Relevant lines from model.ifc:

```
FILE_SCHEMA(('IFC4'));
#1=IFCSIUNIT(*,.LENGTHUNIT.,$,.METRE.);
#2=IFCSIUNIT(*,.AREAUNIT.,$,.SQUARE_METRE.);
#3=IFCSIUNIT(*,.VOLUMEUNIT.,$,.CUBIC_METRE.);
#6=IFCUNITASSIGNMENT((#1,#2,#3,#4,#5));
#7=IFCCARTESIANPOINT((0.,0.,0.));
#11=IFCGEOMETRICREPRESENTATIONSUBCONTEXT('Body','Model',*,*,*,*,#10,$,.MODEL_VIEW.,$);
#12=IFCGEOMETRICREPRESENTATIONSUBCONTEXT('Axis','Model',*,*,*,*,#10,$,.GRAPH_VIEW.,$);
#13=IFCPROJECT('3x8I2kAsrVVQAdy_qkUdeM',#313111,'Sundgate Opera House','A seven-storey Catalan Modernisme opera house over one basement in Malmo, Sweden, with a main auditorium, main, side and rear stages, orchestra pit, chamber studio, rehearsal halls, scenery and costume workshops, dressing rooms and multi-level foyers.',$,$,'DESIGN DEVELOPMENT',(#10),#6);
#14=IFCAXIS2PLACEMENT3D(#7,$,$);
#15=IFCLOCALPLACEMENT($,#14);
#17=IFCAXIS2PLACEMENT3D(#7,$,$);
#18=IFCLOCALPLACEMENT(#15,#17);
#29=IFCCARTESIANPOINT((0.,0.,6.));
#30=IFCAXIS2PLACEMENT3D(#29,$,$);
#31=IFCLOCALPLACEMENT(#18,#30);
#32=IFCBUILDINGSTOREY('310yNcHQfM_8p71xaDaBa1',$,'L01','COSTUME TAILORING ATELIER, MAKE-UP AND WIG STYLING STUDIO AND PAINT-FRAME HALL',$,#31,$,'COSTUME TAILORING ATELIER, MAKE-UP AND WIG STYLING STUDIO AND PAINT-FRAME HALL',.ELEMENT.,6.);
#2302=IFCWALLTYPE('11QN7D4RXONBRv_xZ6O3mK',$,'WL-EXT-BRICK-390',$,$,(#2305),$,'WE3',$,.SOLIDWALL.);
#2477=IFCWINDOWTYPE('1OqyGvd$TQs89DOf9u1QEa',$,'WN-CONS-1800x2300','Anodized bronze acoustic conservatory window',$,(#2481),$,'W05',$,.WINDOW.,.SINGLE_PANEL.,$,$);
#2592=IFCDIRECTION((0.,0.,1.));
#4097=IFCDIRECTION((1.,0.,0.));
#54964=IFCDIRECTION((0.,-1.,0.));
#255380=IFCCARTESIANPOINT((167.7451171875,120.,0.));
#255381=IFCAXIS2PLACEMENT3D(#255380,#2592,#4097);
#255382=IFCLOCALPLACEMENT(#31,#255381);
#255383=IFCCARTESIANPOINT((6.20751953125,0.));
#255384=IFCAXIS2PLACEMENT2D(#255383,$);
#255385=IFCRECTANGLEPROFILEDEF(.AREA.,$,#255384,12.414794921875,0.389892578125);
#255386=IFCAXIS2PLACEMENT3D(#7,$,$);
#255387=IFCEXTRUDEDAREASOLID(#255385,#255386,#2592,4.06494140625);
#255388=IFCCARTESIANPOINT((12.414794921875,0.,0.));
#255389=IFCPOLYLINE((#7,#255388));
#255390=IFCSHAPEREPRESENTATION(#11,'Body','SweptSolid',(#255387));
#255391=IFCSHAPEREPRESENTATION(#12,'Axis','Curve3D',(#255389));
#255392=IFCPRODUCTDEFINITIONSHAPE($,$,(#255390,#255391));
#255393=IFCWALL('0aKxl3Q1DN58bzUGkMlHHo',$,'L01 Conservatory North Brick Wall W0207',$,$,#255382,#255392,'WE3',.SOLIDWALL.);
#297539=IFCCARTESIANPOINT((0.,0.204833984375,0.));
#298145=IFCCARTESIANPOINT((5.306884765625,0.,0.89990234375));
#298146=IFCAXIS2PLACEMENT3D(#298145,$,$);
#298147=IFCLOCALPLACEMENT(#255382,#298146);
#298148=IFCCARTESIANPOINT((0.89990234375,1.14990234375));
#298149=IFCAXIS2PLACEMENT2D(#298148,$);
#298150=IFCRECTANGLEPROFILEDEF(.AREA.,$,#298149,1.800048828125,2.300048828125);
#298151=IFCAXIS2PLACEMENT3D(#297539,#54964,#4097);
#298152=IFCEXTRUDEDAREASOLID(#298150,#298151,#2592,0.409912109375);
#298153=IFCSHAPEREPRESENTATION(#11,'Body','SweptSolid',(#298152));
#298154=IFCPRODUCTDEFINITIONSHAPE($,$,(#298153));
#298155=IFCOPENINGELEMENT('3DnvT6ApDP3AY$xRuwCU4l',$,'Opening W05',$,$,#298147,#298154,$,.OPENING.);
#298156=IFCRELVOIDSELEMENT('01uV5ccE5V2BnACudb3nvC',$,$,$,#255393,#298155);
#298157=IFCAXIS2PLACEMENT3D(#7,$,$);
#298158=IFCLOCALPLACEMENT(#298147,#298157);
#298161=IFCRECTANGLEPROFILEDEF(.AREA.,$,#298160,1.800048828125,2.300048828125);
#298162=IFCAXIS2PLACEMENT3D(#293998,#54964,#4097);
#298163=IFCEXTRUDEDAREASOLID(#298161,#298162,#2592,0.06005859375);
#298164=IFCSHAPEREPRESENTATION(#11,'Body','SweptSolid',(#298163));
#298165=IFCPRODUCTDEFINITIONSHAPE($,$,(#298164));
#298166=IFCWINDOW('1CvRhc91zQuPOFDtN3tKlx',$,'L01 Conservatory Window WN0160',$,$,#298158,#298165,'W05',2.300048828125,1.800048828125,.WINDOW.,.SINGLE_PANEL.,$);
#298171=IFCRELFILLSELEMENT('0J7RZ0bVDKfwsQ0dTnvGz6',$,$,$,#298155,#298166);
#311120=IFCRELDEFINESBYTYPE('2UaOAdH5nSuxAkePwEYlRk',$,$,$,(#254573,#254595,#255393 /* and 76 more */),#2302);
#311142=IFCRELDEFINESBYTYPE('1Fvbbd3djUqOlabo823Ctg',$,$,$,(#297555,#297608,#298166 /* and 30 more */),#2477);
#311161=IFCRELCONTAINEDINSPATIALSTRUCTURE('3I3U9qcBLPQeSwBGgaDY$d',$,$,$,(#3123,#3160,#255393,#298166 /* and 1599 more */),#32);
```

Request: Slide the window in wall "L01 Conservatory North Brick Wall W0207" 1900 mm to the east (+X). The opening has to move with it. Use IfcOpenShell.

```python
import ifcopenshell
import ifcopenshell.api.geometry
import ifcopenshell.util.placement
import ifcopenshell.util.unit

model = ifcopenshell.open("model.ifc")
unit_scale = ifcopenshell.util.unit.calculate_unit_scale(model)

window = model.by_id(298166)
opening = window.FillsVoids[0].RelatingOpeningElement
wall = opening.VoidsElements[0].RelatingBuildingElement

wall_matrix = ifcopenshell.util.placement.get_local_placement(wall.ObjectPlacement)
shift = wall_matrix[:3, 0] * 1.9 / unit_scale
before = ifcopenshell.util.placement.get_local_placement(window.ObjectPlacement)[:3, 3].copy()

# The window is placed relative to its opening, so it follows when the opening moves.
matrix = ifcopenshell.util.placement.get_local_placement(opening.ObjectPlacement)
matrix[:3, 3] += shift
ifcopenshell.api.geometry.edit_object_placement(
    model, product=opening, matrix=matrix, is_si=False, should_transform_children=True
)

after = ifcopenshell.util.placement.get_local_placement(window.ObjectPlacement)[:3, 3]
print("window moved by", (after - before).round(3) + 0.0)

model.write("model-out.ifc")
```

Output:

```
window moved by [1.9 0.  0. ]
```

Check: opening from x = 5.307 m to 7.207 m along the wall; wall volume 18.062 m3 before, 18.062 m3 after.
